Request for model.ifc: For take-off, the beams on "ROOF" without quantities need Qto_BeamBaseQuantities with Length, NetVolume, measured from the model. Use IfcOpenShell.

First a look at what the model holds.

```python
import ifcopenshell
import ifcopenshell.util.element
import ifcopenshell.util.unit

model = ifcopenshell.open("model.ifc")
print(model.schema)
for unit_type in ("LENGTHUNIT", "AREAUNIT", "VOLUMEUNIT"):
    print(unit_type, ifcopenshell.util.unit.calculate_unit_scale(model, unit_type))
storey = next(s for s in model.by_type("IfcBuildingStorey") if s.Name == "ROOF")
beams = [e for e in ifcopenshell.util.element.get_decomposition(storey) if e.is_a("IfcBeam")]
for e in sorted(beams, key=lambda e: e.id()):
    print(e.id(), e.is_a(), e.Name, list(ifcopenshell.util.element.get_psets(e, qtos_only=True)), sep=" | ")
```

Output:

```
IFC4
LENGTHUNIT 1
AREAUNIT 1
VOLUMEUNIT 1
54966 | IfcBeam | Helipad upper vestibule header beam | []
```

```python
import ifcopenshell
import ifcopenshell.api.pset
import ifcopenshell.geom
import ifcopenshell.util.element
import ifcopenshell.util.shape
import ifcopenshell.util.unit

model = ifcopenshell.open("model.ifc")
unit_scale = ifcopenshell.util.unit.calculate_unit_scale(model)
volume_scale = ifcopenshell.util.unit.calculate_unit_scale(model, "VOLUMEUNIT")
settings = ifcopenshell.geom.settings()

storey = next(s for s in model.by_type("IfcBuildingStorey") if s.Name == "ROOF")
beams = [e for e in ifcopenshell.util.element.get_decomposition(storey) if e.is_a("IfcBeam")]

for e in sorted(beams, key=lambda e: e.id()):
    if ifcopenshell.util.element.get_psets(e, qtos_only=True, should_inherit=False):
        continue
    # Geometry comes back in metres, in the element's own axes.
    shape = ifcopenshell.geom.create_shape(settings, e)
    values = {
        "Length": ifcopenshell.util.shape.get_max_xyz(shape.geometry) / unit_scale,
        "NetVolume": ifcopenshell.util.shape.get_volume(shape.geometry) / volume_scale,
    }
    qto = ifcopenshell.api.pset.add_qto(model, product=e, name="Qto_BeamBaseQuantities")
    ifcopenshell.api.pset.edit_qto(model, qto=qto, properties=values)
    print(e.id(), {k: round(v, 3) for k, v in values.items()})

model.write("model_updated.ifc")
```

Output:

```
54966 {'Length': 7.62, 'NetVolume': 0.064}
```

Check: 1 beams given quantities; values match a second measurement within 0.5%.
